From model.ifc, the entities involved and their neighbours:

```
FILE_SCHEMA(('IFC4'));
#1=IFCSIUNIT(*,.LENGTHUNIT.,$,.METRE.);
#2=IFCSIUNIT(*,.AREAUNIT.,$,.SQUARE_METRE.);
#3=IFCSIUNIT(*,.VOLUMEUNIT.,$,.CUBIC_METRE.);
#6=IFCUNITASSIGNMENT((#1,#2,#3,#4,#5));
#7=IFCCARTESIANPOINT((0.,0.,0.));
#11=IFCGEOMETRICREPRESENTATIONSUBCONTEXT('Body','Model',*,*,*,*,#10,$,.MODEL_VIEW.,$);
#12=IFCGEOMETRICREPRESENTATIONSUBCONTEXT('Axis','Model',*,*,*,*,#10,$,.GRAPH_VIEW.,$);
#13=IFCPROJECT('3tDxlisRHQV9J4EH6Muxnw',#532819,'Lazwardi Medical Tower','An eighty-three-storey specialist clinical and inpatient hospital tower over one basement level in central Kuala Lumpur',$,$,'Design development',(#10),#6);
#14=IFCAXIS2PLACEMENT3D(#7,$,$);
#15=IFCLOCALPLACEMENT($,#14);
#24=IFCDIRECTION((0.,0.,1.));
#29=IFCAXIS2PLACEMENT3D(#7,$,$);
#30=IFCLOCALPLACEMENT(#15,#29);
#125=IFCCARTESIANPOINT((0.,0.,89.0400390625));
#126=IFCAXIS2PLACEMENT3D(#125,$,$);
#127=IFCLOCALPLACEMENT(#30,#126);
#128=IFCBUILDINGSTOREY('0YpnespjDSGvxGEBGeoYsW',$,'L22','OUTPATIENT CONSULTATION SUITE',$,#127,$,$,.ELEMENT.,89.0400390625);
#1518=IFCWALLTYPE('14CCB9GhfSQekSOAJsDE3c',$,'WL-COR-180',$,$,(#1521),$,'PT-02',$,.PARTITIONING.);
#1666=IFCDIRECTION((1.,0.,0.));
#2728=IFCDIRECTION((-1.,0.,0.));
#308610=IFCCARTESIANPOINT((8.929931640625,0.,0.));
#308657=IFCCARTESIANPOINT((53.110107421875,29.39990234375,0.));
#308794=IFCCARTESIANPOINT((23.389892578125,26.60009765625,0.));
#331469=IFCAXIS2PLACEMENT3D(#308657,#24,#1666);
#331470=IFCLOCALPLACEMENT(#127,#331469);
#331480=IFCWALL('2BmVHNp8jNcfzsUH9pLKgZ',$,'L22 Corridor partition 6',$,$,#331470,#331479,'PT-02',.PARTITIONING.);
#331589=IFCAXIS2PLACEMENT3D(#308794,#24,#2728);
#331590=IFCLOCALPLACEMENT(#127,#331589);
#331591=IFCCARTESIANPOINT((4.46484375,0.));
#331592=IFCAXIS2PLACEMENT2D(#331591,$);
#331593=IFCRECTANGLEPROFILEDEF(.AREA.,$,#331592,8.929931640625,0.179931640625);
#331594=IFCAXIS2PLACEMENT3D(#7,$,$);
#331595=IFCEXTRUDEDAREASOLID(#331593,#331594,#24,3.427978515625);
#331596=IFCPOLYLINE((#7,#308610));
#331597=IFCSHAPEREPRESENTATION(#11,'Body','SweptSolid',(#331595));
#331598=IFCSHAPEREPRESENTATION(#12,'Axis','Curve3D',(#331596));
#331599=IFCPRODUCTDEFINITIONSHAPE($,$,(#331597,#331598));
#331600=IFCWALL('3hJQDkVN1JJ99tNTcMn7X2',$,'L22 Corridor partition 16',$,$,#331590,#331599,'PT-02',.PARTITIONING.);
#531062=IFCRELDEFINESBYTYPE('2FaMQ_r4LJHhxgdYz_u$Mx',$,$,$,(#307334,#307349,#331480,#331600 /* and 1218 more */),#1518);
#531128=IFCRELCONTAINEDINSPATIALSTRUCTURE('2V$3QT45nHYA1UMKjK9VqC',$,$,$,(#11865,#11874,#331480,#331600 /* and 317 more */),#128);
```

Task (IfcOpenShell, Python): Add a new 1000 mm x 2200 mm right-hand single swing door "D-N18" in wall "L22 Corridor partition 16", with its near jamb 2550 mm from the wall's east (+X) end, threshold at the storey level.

```python
import numpy as np
import ifcopenshell
import ifcopenshell.api.feature
import ifcopenshell.api.geometry
import ifcopenshell.api.root
import ifcopenshell.api.spatial
import ifcopenshell.geom
import ifcopenshell.util.element
import ifcopenshell.util.placement
import ifcopenshell.util.representation
import ifcopenshell.util.shape
import ifcopenshell.util.unit

model = ifcopenshell.open("model.ifc")
unit_scale = ifcopenshell.util.unit.calculate_unit_scale(model)
settings = ifcopenshell.geom.settings()


def volume(element):
    """Net volume in cubic metres, openings subtracted."""
    shape = ifcopenshell.geom.create_shape(settings, element)
    return ifcopenshell.util.shape.get_volume(shape.geometry)


wall = model.by_guid("3hJQDkVN1JJ99tNTcMn7X2")
storey = ifcopenshell.util.element.get_container(wall, ifc_class="IfcBuildingStorey")
context = ifcopenshell.util.representation.get_context(model, "Model", "Body", "MODEL_VIEW")
before = volume(wall)

width, height, from_end, sill = 1, 2.2, 2.55, 0.0  # metres

# The wall runs along its own X axis, and the end named is its -X end.
wall_shape = ifcopenshell.geom.create_shape(settings, wall)
x, y, z = ifcopenshell.util.shape.get_vertices(wall_shape.geometry).T
start = x.min() + from_end
face, thickness = float(y.min()), float(y.max() - y.min())
wall_matrix = ifcopenshell.util.placement.get_local_placement(wall.ObjectPlacement)
level = ifcopenshell.util.placement.get_local_placement(storey.ObjectPlacement)[2, 3]


def in_wall(x, y):
    """Placement at x, y metres in the wall's axes, at sill height."""
    matrix = wall_matrix.copy()
    matrix[:, 3] = wall_matrix @ np.array([x / unit_scale, y / unit_scale, 0.0, 1.0])
    matrix[2, 3] = level + sill / unit_scale
    return matrix


# Opening: a box that overshoots both wall faces by 50 mm.
opening = ifcopenshell.api.root.create_entity(model, ifc_class="IfcOpeningElement", predefined_type="OPENING")
box = ifcopenshell.api.geometry.add_wall_representation(
    model, context=context, length=width, height=height, thickness=thickness + 0.1
)
ifcopenshell.api.geometry.assign_representation(model, product=opening, representation=box)
ifcopenshell.api.geometry.edit_object_placement(model, product=opening, matrix=in_wall(start, face - 0.05), is_si=False)
ifcopenshell.api.feature.add_feature(model, feature=opening, element=wall)

door = ifcopenshell.api.root.create_entity(model, ifc_class="IfcDoor", name="D-N18", predefined_type="DOOR")
door.OverallWidth, door.OverallHeight = width / unit_scale, height / unit_scale
door.OperationType = "SINGLE_SWING_RIGHT"
body = ifcopenshell.api.geometry.add_door_representation(
    model,
    context=context,
    overall_width=door.OverallWidth,
    overall_height=door.OverallHeight,
    operation_type="SINGLE_SWING_RIGHT",
    lining_properties={"LiningDepth": thickness / unit_scale, "ThresholdDepth": thickness / unit_scale},
)
ifcopenshell.api.geometry.assign_representation(model, product=door, representation=body)
ifcopenshell.api.spatial.assign_container(model, products=[door], relating_structure=storey)
ifcopenshell.api.feature.add_filling(model, opening=opening, element=door)

# The lining spans the wall, so the door starts at the wall face.
ifcopenshell.api.geometry.edit_object_placement(model, product=door, matrix=in_wall(start, face), is_si=False)

after = volume(wall)

print(f"wall volume {before:.3f} -> {after:.3f} m3")

model.write("model_edited.ifc")
```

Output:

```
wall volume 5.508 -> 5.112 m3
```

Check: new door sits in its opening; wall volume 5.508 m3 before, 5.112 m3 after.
